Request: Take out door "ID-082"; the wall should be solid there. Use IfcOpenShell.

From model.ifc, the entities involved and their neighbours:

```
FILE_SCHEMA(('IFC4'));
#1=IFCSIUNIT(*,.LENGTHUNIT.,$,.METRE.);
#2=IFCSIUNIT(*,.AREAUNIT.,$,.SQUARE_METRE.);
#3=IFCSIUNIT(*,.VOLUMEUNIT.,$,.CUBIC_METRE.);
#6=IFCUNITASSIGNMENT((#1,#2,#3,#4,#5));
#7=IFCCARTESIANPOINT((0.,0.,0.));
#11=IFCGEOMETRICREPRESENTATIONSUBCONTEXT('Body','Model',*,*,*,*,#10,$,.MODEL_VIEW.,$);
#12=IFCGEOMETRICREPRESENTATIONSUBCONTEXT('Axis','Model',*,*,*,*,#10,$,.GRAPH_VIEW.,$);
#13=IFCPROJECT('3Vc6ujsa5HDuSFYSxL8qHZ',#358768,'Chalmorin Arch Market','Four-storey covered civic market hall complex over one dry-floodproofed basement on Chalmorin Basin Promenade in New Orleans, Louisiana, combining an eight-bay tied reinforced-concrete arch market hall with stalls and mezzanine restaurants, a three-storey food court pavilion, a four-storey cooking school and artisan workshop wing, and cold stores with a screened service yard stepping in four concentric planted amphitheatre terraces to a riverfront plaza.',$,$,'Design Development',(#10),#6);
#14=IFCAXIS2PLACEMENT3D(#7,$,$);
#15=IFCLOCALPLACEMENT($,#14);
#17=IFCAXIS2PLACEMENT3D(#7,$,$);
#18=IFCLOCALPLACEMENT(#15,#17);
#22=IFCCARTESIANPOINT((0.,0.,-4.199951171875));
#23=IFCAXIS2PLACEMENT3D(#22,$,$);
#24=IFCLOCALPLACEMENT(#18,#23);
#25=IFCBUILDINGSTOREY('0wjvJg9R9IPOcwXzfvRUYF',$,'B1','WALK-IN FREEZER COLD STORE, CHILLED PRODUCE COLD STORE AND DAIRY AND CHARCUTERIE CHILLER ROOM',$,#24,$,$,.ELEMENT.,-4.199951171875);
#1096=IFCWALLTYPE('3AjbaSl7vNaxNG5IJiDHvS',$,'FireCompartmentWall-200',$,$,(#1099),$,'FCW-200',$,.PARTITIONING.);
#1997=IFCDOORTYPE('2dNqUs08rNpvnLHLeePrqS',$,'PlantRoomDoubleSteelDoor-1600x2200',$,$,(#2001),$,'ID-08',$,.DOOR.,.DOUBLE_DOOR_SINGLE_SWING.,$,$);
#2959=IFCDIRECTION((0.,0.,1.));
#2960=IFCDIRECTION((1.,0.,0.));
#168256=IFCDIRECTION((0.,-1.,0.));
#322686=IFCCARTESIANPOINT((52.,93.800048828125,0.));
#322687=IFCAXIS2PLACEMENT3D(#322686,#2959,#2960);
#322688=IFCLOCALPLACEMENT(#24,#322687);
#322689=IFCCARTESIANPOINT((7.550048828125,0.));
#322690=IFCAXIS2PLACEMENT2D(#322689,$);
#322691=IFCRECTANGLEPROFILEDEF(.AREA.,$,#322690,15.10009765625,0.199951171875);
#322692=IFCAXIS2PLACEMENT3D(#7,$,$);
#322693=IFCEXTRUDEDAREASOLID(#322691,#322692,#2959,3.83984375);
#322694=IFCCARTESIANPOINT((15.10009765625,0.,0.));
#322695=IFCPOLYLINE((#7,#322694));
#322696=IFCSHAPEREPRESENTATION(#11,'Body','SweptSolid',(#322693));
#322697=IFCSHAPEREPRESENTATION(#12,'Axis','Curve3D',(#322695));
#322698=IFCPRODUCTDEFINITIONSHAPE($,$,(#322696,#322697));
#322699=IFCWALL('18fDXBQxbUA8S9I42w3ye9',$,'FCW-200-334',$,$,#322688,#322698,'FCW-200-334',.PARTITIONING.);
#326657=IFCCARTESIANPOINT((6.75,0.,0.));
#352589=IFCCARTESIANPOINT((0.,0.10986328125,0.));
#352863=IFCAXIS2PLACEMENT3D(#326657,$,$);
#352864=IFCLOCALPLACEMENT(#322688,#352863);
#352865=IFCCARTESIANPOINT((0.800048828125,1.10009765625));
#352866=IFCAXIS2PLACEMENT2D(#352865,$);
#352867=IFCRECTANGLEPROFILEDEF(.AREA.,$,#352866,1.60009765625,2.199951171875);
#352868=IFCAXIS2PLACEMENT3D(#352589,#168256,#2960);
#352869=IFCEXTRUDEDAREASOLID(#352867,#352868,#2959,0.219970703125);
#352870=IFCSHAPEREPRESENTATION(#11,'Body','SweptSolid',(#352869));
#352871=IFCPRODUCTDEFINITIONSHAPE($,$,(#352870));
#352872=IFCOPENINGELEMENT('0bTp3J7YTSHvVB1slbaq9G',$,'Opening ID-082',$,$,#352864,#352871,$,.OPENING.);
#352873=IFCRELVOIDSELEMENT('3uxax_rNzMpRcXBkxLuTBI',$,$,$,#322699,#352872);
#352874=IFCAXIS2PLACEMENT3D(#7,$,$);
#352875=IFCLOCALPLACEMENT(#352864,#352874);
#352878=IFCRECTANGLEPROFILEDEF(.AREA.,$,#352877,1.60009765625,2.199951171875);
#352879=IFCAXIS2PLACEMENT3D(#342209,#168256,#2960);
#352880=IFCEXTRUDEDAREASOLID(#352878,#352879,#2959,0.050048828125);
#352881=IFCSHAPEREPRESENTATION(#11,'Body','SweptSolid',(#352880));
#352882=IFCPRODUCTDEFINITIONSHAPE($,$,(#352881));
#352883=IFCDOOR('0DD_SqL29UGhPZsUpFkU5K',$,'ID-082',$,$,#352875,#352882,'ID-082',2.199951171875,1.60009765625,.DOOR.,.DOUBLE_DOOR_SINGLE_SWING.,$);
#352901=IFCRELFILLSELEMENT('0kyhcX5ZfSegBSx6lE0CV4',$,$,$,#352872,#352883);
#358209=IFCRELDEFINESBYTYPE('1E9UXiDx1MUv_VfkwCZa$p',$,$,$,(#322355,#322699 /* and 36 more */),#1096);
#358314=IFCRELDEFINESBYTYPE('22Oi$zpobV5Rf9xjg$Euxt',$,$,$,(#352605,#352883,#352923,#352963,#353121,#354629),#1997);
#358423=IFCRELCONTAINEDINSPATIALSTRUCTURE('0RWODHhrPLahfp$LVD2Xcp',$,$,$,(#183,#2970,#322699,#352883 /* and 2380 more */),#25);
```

```python
import ifcopenshell
import ifcopenshell.api.feature
import ifcopenshell.api.root
import ifcopenshell.geom
import ifcopenshell.util.shape

model = ifcopenshell.open("model.ifc")
settings = ifcopenshell.geom.settings()


def volume(element):
    """Net volume in cubic metres, openings subtracted."""
    shape = ifcopenshell.geom.create_shape(settings, element)
    return ifcopenshell.util.shape.get_volume(shape.geometry)


door = model.by_guid("0DD_SqL29UGhPZsUpFkU5K")
opening = door.FillsVoids[0].RelatingOpeningElement
wall = opening.VoidsElements[0].RelatingBuildingElement
before = volume(wall)

ifcopenshell.api.root.remove_product(model, product=door)
ifcopenshell.api.feature.remove_feature(model, feature=opening)

after = volume(wall)

print(f"wall volume {before:.3f} -> {after:.3f} m3")

model.write("model_edited.ifc")
```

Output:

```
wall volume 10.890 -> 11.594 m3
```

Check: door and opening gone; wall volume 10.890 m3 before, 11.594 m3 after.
